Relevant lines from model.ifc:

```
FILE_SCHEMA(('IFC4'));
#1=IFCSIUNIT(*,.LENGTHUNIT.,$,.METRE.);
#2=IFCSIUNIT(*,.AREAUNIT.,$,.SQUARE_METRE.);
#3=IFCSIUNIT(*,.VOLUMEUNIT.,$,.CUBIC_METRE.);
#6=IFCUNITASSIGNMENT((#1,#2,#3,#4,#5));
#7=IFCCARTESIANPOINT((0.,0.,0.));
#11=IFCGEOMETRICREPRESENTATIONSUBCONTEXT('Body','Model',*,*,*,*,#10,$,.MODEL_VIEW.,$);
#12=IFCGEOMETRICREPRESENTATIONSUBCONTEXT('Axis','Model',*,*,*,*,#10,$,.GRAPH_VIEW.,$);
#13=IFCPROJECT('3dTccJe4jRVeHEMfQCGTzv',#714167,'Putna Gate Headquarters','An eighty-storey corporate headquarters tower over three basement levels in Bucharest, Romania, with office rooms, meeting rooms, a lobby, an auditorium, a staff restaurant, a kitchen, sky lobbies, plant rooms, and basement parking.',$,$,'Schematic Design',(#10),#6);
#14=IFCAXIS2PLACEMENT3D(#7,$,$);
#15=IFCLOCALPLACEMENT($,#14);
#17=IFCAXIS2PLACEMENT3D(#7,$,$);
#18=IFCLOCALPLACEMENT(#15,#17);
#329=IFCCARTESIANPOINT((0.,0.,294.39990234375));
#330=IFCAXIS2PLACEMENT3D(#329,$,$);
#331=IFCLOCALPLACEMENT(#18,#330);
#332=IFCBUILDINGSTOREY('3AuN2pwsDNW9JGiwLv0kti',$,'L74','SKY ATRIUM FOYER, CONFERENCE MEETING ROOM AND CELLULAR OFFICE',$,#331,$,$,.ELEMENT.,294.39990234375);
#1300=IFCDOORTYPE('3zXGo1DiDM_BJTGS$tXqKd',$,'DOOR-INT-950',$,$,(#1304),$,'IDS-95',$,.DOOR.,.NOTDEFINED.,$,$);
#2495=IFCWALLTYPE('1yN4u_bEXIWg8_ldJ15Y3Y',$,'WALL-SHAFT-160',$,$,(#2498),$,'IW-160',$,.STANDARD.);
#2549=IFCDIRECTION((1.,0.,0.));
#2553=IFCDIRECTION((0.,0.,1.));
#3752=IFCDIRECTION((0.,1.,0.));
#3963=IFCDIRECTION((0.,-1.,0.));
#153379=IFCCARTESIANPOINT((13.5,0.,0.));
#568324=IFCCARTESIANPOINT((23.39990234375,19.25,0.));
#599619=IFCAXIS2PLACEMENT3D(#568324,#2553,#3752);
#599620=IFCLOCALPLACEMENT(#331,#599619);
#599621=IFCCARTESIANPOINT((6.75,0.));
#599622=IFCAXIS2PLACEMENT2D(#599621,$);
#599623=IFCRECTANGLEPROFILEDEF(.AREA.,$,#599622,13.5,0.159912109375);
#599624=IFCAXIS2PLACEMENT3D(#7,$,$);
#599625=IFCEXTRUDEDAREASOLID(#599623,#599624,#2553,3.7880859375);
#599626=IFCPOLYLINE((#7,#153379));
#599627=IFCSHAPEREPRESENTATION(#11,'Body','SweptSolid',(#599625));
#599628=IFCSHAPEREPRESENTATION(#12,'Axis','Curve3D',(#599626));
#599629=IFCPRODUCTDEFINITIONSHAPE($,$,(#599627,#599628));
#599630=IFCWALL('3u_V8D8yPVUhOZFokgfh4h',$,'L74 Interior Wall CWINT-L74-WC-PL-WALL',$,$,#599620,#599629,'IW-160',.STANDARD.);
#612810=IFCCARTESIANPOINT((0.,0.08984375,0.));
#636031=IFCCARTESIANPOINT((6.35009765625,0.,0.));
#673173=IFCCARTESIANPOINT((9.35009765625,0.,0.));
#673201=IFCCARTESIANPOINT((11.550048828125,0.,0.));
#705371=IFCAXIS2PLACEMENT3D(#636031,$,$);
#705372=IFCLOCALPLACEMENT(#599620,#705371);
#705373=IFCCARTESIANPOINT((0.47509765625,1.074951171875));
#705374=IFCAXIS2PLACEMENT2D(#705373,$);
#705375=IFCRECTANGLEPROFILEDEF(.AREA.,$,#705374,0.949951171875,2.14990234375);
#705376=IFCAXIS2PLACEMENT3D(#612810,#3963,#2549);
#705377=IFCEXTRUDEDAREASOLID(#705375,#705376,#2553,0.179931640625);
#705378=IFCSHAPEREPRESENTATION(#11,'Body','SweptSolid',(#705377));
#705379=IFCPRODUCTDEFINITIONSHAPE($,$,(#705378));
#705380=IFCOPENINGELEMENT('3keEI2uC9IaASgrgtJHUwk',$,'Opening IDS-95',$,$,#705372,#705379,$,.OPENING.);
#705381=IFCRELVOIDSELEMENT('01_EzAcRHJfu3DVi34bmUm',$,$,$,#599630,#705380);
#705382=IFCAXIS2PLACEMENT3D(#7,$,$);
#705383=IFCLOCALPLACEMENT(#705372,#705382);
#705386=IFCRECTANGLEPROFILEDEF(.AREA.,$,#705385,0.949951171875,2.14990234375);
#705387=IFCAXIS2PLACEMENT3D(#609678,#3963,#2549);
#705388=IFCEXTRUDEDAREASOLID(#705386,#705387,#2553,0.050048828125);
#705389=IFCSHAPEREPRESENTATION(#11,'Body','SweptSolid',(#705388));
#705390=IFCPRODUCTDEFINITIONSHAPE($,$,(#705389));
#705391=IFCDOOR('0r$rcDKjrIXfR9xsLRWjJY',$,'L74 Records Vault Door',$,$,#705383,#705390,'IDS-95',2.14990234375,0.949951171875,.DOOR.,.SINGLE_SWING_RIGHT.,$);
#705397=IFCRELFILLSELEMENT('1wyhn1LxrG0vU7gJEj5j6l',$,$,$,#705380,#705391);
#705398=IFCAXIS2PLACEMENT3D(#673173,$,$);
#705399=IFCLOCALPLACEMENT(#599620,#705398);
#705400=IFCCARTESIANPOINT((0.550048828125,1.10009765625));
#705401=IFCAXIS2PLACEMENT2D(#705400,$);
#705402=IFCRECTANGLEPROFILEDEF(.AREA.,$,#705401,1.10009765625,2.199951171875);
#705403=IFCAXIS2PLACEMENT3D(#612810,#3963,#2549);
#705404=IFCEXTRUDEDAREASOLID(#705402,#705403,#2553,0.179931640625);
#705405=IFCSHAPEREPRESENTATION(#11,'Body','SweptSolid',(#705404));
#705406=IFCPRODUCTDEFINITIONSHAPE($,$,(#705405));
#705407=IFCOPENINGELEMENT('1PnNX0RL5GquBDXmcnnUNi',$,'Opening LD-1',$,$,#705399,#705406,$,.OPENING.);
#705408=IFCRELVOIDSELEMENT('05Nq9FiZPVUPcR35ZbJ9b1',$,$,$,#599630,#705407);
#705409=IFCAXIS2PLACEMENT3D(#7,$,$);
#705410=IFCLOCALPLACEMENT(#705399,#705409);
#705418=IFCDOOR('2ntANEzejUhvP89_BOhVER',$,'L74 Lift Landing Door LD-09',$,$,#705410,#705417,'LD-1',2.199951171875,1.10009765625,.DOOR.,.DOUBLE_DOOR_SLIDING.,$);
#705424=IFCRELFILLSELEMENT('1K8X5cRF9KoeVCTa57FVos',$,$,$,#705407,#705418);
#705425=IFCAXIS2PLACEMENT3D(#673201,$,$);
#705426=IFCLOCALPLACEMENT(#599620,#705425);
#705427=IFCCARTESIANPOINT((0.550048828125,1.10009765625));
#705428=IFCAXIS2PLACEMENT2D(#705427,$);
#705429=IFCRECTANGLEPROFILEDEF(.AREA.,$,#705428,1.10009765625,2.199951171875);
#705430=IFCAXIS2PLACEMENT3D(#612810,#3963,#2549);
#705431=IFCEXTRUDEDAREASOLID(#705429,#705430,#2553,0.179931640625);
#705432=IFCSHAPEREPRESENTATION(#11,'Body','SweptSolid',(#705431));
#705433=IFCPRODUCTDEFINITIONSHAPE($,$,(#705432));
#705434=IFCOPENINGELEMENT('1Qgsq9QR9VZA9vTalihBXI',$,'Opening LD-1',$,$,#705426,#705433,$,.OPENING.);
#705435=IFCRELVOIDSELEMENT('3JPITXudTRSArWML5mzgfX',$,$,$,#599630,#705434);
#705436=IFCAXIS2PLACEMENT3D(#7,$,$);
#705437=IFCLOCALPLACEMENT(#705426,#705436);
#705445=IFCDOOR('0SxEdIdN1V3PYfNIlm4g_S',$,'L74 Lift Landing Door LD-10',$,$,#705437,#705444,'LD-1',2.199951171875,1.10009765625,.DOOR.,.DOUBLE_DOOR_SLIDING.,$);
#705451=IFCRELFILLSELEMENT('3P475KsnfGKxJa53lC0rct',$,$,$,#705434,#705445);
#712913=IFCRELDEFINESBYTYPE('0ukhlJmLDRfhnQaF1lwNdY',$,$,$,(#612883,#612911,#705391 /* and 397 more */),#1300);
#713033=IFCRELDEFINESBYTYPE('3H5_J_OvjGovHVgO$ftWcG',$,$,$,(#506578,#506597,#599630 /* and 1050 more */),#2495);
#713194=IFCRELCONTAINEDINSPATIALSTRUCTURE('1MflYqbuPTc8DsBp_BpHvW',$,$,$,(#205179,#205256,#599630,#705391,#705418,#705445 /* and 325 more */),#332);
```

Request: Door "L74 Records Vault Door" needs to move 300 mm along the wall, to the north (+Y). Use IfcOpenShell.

```python
import ifcopenshell
import ifcopenshell.api.geometry
import ifcopenshell.util.placement
import ifcopenshell.util.unit

model = ifcopenshell.open("model.ifc")
unit_scale = ifcopenshell.util.unit.calculate_unit_scale(model)

door = model.by_guid("0r$rcDKjrIXfR9xsLRWjJY")
opening = door.FillsVoids[0].RelatingOpeningElement
wall = opening.VoidsElements[0].RelatingBuildingElement

wall_matrix = ifcopenshell.util.placement.get_local_placement(wall.ObjectPlacement)
shift = wall_matrix[:3, 0] * 0.3 / unit_scale
before = ifcopenshell.util.placement.get_local_placement(door.ObjectPlacement)[:3, 3].copy()

# The door is placed relative to its opening, so it follows when the opening moves.
matrix = ifcopenshell.util.placement.get_local_placement(opening.ObjectPlacement)
matrix[:3, 3] += shift
ifcopenshell.api.geometry.edit_object_placement(
    model, product=opening, matrix=matrix, is_si=False, should_transform_children=True
)

after = ifcopenshell.util.placement.get_local_placement(door.ObjectPlacement)[:3, 3]
print("door moved by", (after - before).round(3) + 0.0)

model.write("model_v2.ifc")
```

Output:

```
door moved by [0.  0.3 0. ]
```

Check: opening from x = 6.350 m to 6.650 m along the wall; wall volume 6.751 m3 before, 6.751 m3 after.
